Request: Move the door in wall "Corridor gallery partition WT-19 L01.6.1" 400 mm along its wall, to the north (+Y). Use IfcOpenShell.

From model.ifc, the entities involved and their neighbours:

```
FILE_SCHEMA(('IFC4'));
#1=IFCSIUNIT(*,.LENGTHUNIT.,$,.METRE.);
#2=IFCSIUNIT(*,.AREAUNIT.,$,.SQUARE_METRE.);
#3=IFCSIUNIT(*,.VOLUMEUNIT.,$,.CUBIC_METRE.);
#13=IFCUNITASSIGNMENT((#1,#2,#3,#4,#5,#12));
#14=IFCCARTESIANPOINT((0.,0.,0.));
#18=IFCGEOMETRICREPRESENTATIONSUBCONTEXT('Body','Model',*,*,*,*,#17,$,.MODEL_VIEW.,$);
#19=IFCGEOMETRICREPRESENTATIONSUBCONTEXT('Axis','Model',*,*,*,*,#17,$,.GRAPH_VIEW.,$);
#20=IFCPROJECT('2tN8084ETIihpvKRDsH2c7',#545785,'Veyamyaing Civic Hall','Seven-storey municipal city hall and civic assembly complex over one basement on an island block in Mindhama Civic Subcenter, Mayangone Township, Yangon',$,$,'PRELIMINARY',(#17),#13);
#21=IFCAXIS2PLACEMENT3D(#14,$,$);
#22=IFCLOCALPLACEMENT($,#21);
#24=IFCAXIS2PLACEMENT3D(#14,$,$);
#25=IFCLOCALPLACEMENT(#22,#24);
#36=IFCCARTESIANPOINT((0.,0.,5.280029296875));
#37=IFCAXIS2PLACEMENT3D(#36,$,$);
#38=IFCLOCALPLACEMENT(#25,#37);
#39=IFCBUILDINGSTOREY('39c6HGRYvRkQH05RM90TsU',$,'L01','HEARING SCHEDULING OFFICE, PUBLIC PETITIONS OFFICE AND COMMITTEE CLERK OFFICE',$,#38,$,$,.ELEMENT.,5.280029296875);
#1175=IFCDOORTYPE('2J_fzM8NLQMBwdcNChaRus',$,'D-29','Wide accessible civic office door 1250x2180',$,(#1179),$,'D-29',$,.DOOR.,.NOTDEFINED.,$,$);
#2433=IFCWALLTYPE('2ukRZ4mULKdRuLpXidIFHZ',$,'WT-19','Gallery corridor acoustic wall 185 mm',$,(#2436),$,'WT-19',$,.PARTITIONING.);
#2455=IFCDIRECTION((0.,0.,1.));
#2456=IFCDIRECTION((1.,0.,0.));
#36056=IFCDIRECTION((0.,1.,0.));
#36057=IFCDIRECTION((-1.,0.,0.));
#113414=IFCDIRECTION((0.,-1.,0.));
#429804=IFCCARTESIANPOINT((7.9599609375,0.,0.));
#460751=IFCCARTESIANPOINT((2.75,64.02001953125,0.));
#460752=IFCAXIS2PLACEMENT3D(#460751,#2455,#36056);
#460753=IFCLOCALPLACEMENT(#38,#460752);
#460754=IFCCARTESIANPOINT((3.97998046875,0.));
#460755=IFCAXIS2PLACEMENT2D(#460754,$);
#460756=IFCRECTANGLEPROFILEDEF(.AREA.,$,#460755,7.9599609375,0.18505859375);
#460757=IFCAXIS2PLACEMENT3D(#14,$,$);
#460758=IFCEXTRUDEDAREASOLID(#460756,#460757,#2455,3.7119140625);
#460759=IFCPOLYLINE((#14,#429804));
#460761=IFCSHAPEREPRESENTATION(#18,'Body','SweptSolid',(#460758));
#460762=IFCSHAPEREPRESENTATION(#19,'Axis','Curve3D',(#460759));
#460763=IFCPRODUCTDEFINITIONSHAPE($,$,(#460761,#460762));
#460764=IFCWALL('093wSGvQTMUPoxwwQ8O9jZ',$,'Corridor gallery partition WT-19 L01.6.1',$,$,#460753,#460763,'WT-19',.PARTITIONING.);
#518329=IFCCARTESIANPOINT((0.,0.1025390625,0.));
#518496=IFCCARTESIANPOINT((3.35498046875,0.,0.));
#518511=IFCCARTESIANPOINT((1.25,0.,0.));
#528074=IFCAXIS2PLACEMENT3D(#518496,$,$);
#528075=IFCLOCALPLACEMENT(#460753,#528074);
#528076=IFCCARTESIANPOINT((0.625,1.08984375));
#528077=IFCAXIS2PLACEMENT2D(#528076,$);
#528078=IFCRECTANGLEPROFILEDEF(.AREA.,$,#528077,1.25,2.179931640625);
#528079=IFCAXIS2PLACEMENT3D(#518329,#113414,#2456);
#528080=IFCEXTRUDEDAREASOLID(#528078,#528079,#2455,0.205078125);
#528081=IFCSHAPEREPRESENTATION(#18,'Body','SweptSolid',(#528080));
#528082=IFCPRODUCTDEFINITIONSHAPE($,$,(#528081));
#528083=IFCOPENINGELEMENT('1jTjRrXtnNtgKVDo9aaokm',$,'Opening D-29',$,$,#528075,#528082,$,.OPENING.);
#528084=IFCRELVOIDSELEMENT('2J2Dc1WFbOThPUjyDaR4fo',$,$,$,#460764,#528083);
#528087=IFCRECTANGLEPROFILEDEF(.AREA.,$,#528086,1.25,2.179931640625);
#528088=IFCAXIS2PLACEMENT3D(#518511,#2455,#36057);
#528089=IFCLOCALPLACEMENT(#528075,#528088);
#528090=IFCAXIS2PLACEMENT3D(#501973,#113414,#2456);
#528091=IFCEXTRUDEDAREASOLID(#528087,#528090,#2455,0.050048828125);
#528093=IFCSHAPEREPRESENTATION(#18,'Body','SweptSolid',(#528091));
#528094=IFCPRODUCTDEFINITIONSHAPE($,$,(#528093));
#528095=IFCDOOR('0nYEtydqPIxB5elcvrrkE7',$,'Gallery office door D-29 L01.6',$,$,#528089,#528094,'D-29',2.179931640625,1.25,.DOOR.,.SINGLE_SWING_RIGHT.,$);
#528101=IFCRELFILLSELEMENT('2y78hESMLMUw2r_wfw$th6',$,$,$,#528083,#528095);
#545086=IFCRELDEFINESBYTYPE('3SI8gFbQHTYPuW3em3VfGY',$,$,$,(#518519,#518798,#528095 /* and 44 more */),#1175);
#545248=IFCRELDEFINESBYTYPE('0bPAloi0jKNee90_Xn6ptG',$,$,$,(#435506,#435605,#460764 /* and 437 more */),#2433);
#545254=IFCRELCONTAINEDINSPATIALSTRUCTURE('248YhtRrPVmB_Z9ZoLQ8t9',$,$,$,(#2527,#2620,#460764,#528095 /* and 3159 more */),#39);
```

```python
import ifcopenshell
import ifcopenshell.api.geometry
import ifcopenshell.util.placement

model = ifcopenshell.open("model.ifc")

door = model.by_guid("0nYEtydqPIxB5elcvrrkE7")
opening = door.FillsVoids[0].RelatingOpeningElement
wall = opening.VoidsElements[0].RelatingBuildingElement

wall_matrix = ifcopenshell.util.placement.get_local_placement(wall.ObjectPlacement)
shift = wall_matrix[:3, 0] * 0.4
before = ifcopenshell.util.placement.get_local_placement(door.ObjectPlacement)[:3, 3].copy()

# The door is placed relative to its opening, so it follows when the opening moves.
matrix = ifcopenshell.util.placement.get_local_placement(opening.ObjectPlacement)
matrix[:3, 3] += shift
ifcopenshell.api.geometry.edit_object_placement(
    model, product=opening, matrix=matrix, is_si=False, should_transform_children=True
)

after = ifcopenshell.util.placement.get_local_placement(door.ObjectPlacement)[:3, 3]
print("door moved by", (after - before).round(3) + 0.0)

model.write("model_v2.ifc")
```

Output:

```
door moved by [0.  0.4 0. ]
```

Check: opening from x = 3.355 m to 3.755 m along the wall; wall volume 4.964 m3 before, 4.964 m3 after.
